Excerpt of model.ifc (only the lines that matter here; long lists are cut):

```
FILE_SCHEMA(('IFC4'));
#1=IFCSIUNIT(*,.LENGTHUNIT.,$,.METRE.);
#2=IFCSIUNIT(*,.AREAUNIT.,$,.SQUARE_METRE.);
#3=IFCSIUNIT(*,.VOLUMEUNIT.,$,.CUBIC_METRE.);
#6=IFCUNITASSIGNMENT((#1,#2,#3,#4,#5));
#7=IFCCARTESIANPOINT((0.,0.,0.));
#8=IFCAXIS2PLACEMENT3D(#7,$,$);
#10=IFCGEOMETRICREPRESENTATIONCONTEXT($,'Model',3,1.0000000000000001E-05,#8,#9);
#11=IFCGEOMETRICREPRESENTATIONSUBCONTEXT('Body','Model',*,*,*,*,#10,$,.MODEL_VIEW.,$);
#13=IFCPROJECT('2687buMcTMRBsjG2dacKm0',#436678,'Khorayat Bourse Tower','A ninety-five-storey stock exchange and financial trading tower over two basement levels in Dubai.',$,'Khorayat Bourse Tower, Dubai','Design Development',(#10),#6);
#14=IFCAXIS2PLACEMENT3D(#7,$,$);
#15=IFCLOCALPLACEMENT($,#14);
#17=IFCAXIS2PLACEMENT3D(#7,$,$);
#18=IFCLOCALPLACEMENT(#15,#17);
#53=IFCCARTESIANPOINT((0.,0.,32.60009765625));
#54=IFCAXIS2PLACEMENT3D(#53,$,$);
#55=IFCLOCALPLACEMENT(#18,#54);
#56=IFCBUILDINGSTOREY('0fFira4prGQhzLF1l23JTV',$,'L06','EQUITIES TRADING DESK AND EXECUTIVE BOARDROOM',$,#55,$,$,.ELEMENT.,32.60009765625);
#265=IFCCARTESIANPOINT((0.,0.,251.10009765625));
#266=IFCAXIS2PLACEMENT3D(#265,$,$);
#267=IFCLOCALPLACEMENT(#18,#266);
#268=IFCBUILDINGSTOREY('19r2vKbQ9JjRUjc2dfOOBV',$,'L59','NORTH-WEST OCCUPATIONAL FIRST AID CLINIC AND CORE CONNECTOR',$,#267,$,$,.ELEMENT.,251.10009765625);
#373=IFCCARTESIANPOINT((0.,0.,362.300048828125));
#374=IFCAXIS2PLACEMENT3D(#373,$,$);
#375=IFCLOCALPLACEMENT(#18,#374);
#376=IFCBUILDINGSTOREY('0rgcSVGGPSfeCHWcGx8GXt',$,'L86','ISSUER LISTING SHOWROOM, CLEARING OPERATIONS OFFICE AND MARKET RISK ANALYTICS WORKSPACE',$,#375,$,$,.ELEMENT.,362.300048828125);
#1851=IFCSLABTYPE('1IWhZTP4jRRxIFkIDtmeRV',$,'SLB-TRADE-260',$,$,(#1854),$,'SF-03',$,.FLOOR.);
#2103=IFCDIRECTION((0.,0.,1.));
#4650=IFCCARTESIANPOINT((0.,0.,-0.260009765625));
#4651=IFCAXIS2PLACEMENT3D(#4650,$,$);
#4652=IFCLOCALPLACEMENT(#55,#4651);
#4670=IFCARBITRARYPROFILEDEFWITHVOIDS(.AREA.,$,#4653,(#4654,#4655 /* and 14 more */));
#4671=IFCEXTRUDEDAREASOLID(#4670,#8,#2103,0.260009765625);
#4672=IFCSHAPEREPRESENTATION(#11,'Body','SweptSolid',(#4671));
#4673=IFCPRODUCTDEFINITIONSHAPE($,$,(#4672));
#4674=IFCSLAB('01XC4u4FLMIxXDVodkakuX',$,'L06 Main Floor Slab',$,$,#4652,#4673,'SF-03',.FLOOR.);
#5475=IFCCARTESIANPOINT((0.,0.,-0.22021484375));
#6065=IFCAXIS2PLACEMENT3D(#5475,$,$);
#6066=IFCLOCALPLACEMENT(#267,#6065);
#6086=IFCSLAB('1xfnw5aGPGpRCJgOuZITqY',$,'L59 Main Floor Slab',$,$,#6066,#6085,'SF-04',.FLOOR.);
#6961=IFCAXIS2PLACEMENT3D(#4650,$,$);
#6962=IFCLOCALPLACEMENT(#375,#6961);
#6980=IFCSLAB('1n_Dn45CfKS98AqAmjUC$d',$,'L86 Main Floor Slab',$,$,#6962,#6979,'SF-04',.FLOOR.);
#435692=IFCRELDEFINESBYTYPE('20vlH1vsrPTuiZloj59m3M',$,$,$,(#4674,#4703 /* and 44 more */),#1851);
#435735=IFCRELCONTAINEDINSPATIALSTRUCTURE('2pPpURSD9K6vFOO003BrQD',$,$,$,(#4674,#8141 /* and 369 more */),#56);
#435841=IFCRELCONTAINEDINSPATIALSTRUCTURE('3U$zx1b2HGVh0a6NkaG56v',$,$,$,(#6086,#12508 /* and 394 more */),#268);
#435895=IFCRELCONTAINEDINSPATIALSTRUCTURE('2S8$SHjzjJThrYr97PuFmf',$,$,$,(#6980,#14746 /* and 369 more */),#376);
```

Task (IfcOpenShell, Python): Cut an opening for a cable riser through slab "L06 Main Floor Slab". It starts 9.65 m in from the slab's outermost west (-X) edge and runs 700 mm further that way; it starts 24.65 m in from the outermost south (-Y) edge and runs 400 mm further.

```python
import numpy as np
import ifcopenshell
import ifcopenshell.api.feature
import ifcopenshell.api.geometry
import ifcopenshell.api.root
import ifcopenshell.geom
import ifcopenshell.util.placement
import ifcopenshell.util.representation
import ifcopenshell.util.shape
import ifcopenshell.util.unit

model = ifcopenshell.open("model.ifc")
unit_scale = ifcopenshell.util.unit.calculate_unit_scale(model)
settings = ifcopenshell.geom.settings()


def volume(element):
    """Net volume in cubic metres, openings subtracted."""
    shape = ifcopenshell.geom.create_shape(settings, element)
    return ifcopenshell.util.shape.get_volume(shape.geometry)


slab = model.by_id(4674)
before = volume(slab)

# Extent in the slab's own axes, in metres. The edges named are its -X and -Y sides.
slab_shape = ifcopenshell.geom.create_shape(settings, slab)
vertices = ifcopenshell.util.shape.get_vertices(slab_shape.geometry)
x_min, y_min, bottom = vertices.min(axis=0)
top = vertices[:, 2].max()

opening = ifcopenshell.api.root.create_entity(model, ifc_class="IfcOpeningElement", name="Cable riser opening", predefined_type="OPENING")
context = ifcopenshell.util.representation.get_context(model, "Model", "Body", "MODEL_VIEW")
width, depth = 0.7, 0.4
outline = [(0.0, 0.0), (width, 0.0), (width, depth), (0.0, depth), (0.0, 0.0)]
# Overshoot both faces by 50 mm so the cut is clean.
shape = ifcopenshell.api.geometry.add_slab_representation(
    model, context=context, depth=top - bottom + 0.1, polyline=outline
)
ifcopenshell.api.geometry.assign_representation(model, product=opening, representation=shape)

matrix = ifcopenshell.util.placement.get_local_placement(slab.ObjectPlacement)
matrix[:, 3] = matrix @ np.append(np.array([x_min + 9.65, y_min + 24.65, bottom - 0.05]) / unit_scale, 1.0)
ifcopenshell.api.geometry.edit_object_placement(model, product=opening, matrix=matrix, is_si=False)
ifcopenshell.api.feature.add_feature(model, feature=opening, element=slab)

after = volume(slab)

print(f"slab volume {before:.3f} -> {after:.3f} m3")

model.write("model-out.ifc")
```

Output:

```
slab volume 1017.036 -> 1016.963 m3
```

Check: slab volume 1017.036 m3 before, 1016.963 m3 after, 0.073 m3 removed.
